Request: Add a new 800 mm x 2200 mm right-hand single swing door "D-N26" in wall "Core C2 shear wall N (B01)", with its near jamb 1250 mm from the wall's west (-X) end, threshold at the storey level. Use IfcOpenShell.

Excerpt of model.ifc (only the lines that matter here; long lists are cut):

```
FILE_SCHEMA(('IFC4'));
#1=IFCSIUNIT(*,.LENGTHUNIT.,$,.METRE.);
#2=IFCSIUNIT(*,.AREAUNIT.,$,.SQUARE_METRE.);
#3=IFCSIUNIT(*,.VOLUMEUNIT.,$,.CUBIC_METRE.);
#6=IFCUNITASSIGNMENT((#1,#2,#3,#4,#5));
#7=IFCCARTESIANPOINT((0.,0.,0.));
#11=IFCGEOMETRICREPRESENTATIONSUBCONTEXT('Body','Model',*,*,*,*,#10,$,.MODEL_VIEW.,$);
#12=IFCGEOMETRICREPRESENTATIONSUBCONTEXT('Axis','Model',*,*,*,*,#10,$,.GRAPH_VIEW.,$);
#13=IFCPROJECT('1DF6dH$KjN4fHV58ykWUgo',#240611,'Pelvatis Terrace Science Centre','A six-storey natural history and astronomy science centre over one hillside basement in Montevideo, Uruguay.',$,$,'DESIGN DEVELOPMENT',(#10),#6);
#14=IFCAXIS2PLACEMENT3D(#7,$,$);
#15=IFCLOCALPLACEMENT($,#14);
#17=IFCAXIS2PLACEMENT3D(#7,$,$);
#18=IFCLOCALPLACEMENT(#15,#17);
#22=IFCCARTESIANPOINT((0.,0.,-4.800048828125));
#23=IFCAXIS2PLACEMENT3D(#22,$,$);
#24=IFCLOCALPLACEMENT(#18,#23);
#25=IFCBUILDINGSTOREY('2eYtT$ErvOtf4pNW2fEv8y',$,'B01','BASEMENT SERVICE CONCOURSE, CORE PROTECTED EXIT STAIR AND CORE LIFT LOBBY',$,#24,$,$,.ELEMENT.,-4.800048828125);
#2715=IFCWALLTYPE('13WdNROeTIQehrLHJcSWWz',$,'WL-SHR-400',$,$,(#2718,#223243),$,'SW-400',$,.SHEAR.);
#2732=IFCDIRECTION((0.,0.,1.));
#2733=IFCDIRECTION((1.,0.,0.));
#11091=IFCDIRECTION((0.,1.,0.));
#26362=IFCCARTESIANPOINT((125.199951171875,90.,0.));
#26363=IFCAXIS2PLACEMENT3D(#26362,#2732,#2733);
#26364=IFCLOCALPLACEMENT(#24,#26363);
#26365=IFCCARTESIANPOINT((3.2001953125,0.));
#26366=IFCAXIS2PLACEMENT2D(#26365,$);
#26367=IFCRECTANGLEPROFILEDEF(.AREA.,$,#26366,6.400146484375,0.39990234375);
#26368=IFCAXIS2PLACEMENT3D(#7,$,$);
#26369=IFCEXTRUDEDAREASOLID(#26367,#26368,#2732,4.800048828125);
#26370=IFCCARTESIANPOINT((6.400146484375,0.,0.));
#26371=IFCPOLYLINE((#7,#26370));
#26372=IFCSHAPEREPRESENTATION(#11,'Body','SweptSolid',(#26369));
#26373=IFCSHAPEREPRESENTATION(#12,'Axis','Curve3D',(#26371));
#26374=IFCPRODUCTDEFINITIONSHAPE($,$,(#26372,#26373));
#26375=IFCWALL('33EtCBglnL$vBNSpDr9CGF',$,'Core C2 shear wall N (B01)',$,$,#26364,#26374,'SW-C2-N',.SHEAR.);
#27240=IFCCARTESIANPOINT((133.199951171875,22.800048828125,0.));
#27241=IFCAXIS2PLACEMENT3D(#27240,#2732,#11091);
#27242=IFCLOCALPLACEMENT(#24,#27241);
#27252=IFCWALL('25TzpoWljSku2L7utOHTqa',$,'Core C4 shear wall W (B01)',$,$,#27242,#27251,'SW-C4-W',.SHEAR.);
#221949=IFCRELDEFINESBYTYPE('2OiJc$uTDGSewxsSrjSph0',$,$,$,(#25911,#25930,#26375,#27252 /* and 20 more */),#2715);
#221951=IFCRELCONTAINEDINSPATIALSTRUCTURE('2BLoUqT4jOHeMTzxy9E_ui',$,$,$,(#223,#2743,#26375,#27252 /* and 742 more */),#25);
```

```python
import numpy as np
import ifcopenshell
import ifcopenshell.api.feature
import ifcopenshell.api.geometry
import ifcopenshell.api.root
import ifcopenshell.api.spatial
import ifcopenshell.geom
import ifcopenshell.util.element
import ifcopenshell.util.placement
import ifcopenshell.util.representation
import ifcopenshell.util.shape
import ifcopenshell.util.unit

model = ifcopenshell.open("model.ifc")
unit_scale = ifcopenshell.util.unit.calculate_unit_scale(model)
settings = ifcopenshell.geom.settings()


def volume(element):
    """Net volume in cubic metres, openings subtracted."""
    shape = ifcopenshell.geom.create_shape(settings, element)
    return ifcopenshell.util.shape.get_volume(shape.geometry)


wall = model.by_guid("33EtCBglnL$vBNSpDr9CGF")
storey = ifcopenshell.util.element.get_container(wall, ifc_class="IfcBuildingStorey")
context = ifcopenshell.util.representation.get_context(model, "Model", "Body", "MODEL_VIEW")
before = volume(wall)

width, height, from_end, sill = 0.8, 2.2, 1.25, 0.0  # metres

# The wall runs along its own X axis, and the end named is its -X end.
wall_shape = ifcopenshell.geom.create_shape(settings, wall)
x, y, z = ifcopenshell.util.shape.get_vertices(wall_shape.geometry).T
start = x.min() + from_end
face, thickness = float(y.min()), float(y.max() - y.min())
wall_matrix = ifcopenshell.util.placement.get_local_placement(wall.ObjectPlacement)
level = ifcopenshell.util.placement.get_local_placement(storey.ObjectPlacement)[2, 3]


def in_wall(x, y):
    """Placement at x, y metres in the wall's axes, at sill height."""
    matrix = wall_matrix.copy()
    matrix[:, 3] = wall_matrix @ np.array([x / unit_scale, y / unit_scale, 0.0, 1.0])
    matrix[2, 3] = level + sill / unit_scale
    return matrix


# Opening: a box that overshoots both wall faces by 50 mm.
opening = ifcopenshell.api.root.create_entity(model, ifc_class="IfcOpeningElement", predefined_type="OPENING")
box = ifcopenshell.api.geometry.add_wall_representation(
    model, context=context, length=width, height=height, thickness=thickness + 0.1
)
ifcopenshell.api.geometry.assign_representation(model, product=opening, representation=box)
ifcopenshell.api.geometry.edit_object_placement(model, product=opening, matrix=in_wall(start, face - 0.05), is_si=False)
ifcopenshell.api.feature.add_feature(model, feature=opening, element=wall)

door = ifcopenshell.api.root.create_entity(model, ifc_class="IfcDoor", name="D-N26", predefined_type="DOOR")
door.OverallWidth, door.OverallHeight = width / unit_scale, height / unit_scale
door.OperationType = "SINGLE_SWING_RIGHT"
body = ifcopenshell.api.geometry.add_door_representation(
    model,
    context=context,
    overall_width=door.OverallWidth,
    overall_height=door.OverallHeight,
    operation_type="SINGLE_SWING_RIGHT",
    lining_properties={"LiningDepth": thickness / unit_scale, "ThresholdDepth": thickness / unit_scale},
)
ifcopenshell.api.geometry.assign_representation(model, product=door, representation=body)
ifcopenshell.api.spatial.assign_container(model, products=[door], relating_structure=storey)
ifcopenshell.api.feature.add_filling(model, opening=opening, element=door)

# The lining spans the wall, so the door starts at the wall face.
ifcopenshell.api.geometry.edit_object_placement(model, product=door, matrix=in_wall(start, face), is_si=False)

after = volume(wall)

print(f"wall volume {before:.3f} -> {after:.3f} m3")

model.write("model-out.ifc")
```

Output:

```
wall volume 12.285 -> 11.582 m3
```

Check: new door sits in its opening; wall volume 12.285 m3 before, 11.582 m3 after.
